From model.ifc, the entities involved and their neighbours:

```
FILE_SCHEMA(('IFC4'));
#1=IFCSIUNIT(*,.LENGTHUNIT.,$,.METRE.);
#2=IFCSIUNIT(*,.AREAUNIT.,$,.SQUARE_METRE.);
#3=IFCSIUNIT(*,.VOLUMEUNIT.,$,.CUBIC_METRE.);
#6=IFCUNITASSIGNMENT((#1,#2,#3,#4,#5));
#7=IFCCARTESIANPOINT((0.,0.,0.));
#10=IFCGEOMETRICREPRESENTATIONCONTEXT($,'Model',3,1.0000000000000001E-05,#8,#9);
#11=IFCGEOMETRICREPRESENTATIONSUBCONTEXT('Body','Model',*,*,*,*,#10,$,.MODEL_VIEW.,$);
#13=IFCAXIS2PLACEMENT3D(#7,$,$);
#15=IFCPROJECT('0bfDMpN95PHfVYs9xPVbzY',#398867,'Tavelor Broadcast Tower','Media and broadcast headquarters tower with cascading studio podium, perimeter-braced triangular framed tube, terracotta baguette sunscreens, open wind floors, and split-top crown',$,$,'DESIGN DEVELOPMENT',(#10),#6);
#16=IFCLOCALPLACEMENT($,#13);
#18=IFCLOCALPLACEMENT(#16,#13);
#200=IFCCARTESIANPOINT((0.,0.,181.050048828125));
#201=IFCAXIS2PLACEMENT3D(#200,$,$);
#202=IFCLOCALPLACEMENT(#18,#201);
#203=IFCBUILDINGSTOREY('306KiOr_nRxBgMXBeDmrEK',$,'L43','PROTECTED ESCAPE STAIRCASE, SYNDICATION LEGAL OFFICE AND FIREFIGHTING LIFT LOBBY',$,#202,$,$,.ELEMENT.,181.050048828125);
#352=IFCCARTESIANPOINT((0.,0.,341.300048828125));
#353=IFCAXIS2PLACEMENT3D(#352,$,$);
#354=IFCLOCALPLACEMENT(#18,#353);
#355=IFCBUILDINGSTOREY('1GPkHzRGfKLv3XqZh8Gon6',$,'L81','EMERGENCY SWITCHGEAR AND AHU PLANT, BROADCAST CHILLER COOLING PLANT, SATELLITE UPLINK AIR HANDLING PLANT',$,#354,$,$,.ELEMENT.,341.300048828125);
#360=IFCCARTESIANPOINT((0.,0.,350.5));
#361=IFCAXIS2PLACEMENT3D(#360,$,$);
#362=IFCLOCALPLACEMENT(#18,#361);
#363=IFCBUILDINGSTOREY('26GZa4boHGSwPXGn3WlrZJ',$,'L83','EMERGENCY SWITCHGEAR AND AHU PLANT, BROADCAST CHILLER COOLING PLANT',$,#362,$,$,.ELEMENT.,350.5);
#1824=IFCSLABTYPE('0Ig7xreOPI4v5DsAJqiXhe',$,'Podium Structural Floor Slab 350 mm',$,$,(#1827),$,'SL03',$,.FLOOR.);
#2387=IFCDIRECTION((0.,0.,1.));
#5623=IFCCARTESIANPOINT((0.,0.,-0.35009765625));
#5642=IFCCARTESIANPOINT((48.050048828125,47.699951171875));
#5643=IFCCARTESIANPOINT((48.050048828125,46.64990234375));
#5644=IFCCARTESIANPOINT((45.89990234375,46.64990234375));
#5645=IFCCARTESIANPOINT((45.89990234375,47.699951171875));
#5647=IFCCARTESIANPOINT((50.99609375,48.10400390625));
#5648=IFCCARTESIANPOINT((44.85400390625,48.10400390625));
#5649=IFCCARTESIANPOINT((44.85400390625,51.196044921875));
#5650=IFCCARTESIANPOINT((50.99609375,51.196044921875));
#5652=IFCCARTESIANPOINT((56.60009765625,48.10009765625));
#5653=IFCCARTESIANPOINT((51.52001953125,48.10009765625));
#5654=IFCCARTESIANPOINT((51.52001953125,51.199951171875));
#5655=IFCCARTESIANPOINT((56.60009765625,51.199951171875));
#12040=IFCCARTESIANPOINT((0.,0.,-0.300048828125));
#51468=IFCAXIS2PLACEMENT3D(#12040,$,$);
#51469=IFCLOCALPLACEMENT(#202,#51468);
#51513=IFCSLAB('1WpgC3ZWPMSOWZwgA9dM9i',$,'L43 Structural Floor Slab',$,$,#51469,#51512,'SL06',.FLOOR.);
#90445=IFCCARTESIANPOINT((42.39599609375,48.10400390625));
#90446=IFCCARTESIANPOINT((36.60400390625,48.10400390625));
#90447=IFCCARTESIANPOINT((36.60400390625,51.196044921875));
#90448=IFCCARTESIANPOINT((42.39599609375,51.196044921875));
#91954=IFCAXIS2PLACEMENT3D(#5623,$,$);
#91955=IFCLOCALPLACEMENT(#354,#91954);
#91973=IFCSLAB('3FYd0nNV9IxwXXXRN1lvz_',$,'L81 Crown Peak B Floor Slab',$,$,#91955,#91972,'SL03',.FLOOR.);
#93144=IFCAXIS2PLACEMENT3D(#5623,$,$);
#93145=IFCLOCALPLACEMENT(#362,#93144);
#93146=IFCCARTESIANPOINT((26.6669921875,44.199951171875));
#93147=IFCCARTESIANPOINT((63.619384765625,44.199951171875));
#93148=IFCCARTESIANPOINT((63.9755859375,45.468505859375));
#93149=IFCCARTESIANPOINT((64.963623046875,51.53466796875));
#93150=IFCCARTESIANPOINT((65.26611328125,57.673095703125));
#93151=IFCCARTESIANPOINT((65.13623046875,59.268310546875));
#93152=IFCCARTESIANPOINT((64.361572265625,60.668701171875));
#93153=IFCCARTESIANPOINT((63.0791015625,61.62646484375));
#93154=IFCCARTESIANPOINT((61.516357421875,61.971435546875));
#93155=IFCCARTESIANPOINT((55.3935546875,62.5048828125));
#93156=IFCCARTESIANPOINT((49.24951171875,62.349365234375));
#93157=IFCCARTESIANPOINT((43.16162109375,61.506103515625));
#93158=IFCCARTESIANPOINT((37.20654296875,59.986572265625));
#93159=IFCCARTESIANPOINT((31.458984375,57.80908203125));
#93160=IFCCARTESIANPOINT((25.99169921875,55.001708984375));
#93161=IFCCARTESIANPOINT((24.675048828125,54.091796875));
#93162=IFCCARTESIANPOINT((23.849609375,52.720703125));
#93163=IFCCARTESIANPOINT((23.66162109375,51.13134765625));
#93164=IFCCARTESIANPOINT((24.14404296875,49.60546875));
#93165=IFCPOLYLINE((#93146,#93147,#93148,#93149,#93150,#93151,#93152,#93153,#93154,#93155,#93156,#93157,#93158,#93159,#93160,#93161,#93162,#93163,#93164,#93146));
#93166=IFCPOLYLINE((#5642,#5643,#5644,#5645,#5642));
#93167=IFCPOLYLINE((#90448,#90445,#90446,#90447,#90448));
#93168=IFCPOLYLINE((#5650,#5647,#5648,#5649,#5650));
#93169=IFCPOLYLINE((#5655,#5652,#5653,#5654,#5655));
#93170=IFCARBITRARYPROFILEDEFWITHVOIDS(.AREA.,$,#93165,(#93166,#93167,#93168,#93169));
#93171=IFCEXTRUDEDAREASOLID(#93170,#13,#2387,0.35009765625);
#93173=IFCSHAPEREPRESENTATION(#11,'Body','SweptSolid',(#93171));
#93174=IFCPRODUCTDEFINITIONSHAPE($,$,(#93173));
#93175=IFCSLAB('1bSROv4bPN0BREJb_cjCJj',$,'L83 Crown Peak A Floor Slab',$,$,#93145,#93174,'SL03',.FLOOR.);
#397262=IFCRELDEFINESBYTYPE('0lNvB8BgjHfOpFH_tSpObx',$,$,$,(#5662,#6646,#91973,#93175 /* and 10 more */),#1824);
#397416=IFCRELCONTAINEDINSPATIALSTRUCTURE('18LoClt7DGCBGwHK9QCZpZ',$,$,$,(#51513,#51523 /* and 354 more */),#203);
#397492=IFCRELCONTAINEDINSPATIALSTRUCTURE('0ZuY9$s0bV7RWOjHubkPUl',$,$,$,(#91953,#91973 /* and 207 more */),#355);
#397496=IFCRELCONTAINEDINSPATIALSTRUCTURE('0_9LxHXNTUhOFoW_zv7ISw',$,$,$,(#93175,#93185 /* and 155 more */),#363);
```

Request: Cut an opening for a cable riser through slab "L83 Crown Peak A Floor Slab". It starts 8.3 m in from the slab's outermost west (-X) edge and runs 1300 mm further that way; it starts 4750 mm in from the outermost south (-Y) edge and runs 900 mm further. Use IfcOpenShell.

```python
import numpy as np
import ifcopenshell
import ifcopenshell.api.feature
import ifcopenshell.api.geometry
import ifcopenshell.api.root
import ifcopenshell.geom
import ifcopenshell.util.placement
import ifcopenshell.util.representation
import ifcopenshell.util.shape
import ifcopenshell.util.unit

model = ifcopenshell.open("model.ifc")
unit_scale = ifcopenshell.util.unit.calculate_unit_scale(model)
settings = ifcopenshell.geom.settings()


def volume(element):
    """Net volume in cubic metres, openings subtracted."""
    shape = ifcopenshell.geom.create_shape(settings, element)
    return ifcopenshell.util.shape.get_volume(shape.geometry)


slab = model.by_id(93175)
before = volume(slab)

# Extent in the slab's own axes, in metres. The edges named are its -X and -Y sides.
slab_shape = ifcopenshell.geom.create_shape(settings, slab)
vertices = ifcopenshell.util.shape.get_vertices(slab_shape.geometry)
x_min, y_min, bottom = vertices.min(axis=0)
top = vertices[:, 2].max()

opening = ifcopenshell.api.root.create_entity(model, ifc_class="IfcOpeningElement", name="Cable riser opening", predefined_type="OPENING")
context = ifcopenshell.util.representation.get_context(model, "Model", "Body", "MODEL_VIEW")
width, depth = 1.3, 0.9
outline = [(0.0, 0.0), (width, 0.0), (width, depth), (0.0, depth), (0.0, 0.0)]
# Overshoot both faces by 50 mm so the cut is clean.
shape = ifcopenshell.api.geometry.add_slab_representation(
    model, context=context, depth=top - bottom + 0.1, polyline=outline
)
ifcopenshell.api.geometry.assign_representation(model, product=opening, representation=shape)

matrix = ifcopenshell.util.placement.get_local_placement(slab.ObjectPlacement)
matrix[:, 3] = matrix @ np.append(np.array([x_min + 8.3, y_min + 4.75, bottom - 0.05]) / unit_scale, 1.0)
ifcopenshell.api.geometry.edit_object_placement(model, product=opening, matrix=matrix, is_si=False)
ifcopenshell.api.feature.add_feature(model, feature=opening, element=slab)

after = volume(slab)

print(f"slab volume {before:.3f} -> {after:.3f} m3")

model.write("model_edited.ifc")
```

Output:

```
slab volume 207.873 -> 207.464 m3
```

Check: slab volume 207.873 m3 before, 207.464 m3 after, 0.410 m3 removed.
